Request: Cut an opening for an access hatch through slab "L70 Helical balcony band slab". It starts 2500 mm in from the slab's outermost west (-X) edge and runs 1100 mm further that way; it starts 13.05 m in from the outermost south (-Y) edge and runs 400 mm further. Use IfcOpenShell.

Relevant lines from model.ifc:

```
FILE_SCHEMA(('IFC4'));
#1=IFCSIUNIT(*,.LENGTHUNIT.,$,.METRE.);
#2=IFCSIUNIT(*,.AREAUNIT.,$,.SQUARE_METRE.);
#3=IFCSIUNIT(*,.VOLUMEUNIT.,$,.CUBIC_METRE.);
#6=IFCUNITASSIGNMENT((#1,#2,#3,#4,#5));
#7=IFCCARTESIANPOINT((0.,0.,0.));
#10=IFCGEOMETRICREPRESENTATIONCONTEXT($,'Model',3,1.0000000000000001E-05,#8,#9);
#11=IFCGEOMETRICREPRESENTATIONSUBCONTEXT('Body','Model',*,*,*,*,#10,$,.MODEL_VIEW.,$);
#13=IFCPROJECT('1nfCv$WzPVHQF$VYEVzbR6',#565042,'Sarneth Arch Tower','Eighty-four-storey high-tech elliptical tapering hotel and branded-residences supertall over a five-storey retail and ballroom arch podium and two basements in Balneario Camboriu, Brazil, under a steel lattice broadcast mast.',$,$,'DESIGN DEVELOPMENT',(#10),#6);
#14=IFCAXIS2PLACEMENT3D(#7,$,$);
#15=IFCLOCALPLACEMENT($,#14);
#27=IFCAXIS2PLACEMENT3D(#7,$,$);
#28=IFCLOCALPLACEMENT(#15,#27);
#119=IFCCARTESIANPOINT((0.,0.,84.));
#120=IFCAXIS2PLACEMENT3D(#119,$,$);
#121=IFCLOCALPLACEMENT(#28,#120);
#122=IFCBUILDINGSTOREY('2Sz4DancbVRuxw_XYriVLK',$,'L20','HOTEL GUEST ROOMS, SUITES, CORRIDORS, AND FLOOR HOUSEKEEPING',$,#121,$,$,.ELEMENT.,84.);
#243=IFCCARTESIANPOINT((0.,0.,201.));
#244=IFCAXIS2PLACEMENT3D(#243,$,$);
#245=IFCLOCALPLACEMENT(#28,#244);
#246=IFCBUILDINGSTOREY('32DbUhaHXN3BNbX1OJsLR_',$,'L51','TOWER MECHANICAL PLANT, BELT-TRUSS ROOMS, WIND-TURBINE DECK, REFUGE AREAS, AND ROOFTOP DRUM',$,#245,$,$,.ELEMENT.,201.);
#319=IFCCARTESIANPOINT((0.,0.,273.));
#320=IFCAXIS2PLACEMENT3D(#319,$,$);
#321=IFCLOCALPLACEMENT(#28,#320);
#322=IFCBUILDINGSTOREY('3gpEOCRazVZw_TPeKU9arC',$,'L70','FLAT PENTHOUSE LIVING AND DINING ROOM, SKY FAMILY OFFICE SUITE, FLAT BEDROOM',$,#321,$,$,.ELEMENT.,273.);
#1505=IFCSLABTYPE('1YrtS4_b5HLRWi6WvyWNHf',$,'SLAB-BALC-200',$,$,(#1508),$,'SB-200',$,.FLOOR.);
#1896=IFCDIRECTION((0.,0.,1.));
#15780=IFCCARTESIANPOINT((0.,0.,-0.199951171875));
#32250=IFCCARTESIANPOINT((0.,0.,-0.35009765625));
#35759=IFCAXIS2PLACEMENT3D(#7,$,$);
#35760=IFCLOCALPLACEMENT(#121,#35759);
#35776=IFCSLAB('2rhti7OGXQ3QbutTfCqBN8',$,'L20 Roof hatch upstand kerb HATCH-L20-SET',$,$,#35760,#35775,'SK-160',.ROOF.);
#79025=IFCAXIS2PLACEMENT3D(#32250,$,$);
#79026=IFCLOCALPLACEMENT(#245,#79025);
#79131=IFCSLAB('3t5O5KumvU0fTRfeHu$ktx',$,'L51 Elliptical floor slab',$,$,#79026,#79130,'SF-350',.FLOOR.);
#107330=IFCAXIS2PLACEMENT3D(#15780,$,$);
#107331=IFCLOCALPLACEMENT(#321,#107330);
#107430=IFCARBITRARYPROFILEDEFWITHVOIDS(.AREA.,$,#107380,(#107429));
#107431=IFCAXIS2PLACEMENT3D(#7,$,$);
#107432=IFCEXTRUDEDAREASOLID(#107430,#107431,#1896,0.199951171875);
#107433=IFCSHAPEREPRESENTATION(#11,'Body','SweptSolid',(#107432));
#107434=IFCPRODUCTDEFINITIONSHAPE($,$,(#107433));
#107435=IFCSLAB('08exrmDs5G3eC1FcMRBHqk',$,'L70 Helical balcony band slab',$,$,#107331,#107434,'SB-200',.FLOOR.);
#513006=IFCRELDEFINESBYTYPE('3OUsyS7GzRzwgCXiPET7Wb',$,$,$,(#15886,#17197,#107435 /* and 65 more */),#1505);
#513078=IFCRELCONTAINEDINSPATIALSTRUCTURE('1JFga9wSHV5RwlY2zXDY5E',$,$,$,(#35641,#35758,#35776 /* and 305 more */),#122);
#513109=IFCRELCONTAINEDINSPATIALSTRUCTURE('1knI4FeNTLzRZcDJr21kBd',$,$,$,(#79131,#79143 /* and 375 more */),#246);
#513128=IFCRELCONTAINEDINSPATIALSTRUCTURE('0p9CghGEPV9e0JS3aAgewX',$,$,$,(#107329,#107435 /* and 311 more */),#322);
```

```python
import numpy as np
import ifcopenshell
import ifcopenshell.api.feature
import ifcopenshell.api.geometry
import ifcopenshell.api.root
import ifcopenshell.geom
import ifcopenshell.util.placement
import ifcopenshell.util.representation
import ifcopenshell.util.shape
import ifcopenshell.util.unit

model = ifcopenshell.open("model.ifc")
unit_scale = ifcopenshell.util.unit.calculate_unit_scale(model)
settings = ifcopenshell.geom.settings()


def volume(element):
    """Net volume in cubic metres, openings subtracted."""
    shape = ifcopenshell.geom.create_shape(settings, element)
    return ifcopenshell.util.shape.get_volume(shape.geometry)


slab = model.by_id(107435)
before = volume(slab)

# Extent in the slab's own axes, in metres. The edges named are its -X and -Y sides.
slab_shape = ifcopenshell.geom.create_shape(settings, slab)
vertices = ifcopenshell.util.shape.get_vertices(slab_shape.geometry)
x_min, y_min, bottom = vertices.min(axis=0)
top = vertices[:, 2].max()

opening = ifcopenshell.api.root.create_entity(model, ifc_class="IfcOpeningElement", name="Access hatch opening", predefined_type="OPENING")
context = ifcopenshell.util.representation.get_context(model, "Model", "Body", "MODEL_VIEW")
width, depth = 1.1, 0.4
outline = [(0.0, 0.0), (width, 0.0), (width, depth), (0.0, depth), (0.0, 0.0)]
# Overshoot both faces by 50 mm so the cut is clean.
shape = ifcopenshell.api.geometry.add_slab_representation(
    model, context=context, depth=top - bottom + 0.1, polyline=outline
)
ifcopenshell.api.geometry.assign_representation(model, product=opening, representation=shape)

matrix = ifcopenshell.util.placement.get_local_placement(slab.ObjectPlacement)
matrix[:, 3] = matrix @ np.append(np.array([x_min + 2.5, y_min + 13.05, bottom - 0.05]) / unit_scale, 1.0)
ifcopenshell.api.geometry.edit_object_placement(model, product=opening, matrix=matrix, is_si=False)
ifcopenshell.api.feature.add_feature(model, feature=opening, element=slab)

after = volume(slab)

print(f"slab volume {before:.3f} -> {after:.3f} m3")

model.write("model_rev.ifc")
```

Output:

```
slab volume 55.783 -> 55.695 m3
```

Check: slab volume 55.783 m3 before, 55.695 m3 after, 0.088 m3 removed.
